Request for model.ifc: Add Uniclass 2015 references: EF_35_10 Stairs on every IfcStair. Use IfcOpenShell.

First a look at what the model holds.

```python
import ifcopenshell

model = ifcopenshell.open("model.ifc")
print(model.schema)
print("classifications:", [c.Name for c in model.by_type("IfcClassification")])
for ifc_class in ("IfcDoor", "IfcRoof", "IfcStair", "IfcWall", "IfcWindow"):
    print(ifc_class, len(model.by_type(ifc_class)))
```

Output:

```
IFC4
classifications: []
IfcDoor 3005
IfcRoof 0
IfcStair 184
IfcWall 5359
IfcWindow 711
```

```python
import ifcopenshell
import ifcopenshell.api.classification

model = ifcopenshell.open("model.ifc")

system = ifcopenshell.api.classification.add_classification(model, classification="Uniclass 2015")

codes = {
    "IfcStair": ("EF_35_10", "Stairs"),
}
for ifc_class, (code, name) in codes.items():
    products = model.by_type(ifc_class)
    ifcopenshell.api.classification.add_reference(
        model, products=products, classification=system, identification=code, name=name
    )
    print(code, len(products))

model.write("model_edited.ifc")
```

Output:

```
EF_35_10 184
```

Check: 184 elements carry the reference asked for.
